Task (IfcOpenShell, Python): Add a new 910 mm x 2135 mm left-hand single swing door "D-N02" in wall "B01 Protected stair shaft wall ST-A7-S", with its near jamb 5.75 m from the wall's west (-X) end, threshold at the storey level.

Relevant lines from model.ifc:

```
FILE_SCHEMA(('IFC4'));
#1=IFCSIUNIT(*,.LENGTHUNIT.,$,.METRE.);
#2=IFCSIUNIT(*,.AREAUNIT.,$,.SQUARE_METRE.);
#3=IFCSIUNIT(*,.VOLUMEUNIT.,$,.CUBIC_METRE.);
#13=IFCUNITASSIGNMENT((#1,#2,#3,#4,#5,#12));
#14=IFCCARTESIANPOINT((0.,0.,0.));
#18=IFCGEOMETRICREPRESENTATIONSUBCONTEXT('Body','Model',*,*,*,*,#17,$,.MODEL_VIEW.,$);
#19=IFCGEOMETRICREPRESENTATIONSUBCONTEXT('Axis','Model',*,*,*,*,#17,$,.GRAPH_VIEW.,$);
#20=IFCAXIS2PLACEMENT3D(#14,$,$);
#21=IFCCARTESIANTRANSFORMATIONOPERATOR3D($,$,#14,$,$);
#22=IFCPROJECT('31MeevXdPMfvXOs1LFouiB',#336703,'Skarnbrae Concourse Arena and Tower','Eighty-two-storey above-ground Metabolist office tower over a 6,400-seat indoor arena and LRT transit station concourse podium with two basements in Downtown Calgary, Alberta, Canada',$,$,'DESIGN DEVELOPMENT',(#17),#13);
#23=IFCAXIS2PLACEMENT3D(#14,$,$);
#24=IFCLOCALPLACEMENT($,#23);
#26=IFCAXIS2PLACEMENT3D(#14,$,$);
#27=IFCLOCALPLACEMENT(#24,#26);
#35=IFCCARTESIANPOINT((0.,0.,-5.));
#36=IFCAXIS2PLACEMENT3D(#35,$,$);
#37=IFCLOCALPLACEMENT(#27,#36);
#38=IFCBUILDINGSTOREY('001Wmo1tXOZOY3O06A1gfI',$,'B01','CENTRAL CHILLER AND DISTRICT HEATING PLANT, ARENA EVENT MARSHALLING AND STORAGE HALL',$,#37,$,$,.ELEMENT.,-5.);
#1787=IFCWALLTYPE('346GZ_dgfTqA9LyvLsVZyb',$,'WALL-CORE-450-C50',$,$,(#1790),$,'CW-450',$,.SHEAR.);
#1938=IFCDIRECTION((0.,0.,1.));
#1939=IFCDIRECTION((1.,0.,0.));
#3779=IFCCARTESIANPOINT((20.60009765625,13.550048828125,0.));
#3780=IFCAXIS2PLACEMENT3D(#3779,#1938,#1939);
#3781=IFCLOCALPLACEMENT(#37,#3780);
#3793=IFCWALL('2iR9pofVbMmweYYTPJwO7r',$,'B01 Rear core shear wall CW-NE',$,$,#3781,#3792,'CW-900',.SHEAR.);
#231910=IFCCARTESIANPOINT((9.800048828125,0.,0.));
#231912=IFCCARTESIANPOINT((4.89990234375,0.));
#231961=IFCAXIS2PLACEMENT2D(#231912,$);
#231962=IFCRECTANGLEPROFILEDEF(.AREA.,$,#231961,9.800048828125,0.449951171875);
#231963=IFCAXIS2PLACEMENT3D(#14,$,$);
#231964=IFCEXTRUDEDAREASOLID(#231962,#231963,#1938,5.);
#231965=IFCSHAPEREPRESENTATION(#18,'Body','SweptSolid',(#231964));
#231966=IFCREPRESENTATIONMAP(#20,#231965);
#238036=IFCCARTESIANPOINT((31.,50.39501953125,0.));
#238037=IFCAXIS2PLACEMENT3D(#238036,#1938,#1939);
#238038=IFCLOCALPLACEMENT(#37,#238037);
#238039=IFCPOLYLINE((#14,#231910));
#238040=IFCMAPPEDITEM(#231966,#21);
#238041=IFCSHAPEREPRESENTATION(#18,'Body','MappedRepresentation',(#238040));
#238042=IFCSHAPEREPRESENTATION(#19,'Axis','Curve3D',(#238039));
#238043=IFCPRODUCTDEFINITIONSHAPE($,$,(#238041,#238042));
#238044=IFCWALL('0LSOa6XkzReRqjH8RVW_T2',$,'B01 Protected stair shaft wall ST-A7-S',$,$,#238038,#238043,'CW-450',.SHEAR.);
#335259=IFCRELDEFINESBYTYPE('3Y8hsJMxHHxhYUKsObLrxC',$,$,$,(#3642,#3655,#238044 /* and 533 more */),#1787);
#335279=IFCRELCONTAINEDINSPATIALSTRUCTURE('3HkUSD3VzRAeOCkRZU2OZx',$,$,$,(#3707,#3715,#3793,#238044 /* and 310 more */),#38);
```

```python
import numpy as np
import ifcopenshell
import ifcopenshell.api.feature
import ifcopenshell.api.geometry
import ifcopenshell.api.root
import ifcopenshell.api.spatial
import ifcopenshell.geom
import ifcopenshell.util.element
import ifcopenshell.util.placement
import ifcopenshell.util.representation
import ifcopenshell.util.shape
import ifcopenshell.util.unit

model = ifcopenshell.open("model.ifc")
unit_scale = ifcopenshell.util.unit.calculate_unit_scale(model)
settings = ifcopenshell.geom.settings()


def volume(element):
    """Net volume in cubic metres, openings subtracted."""
    shape = ifcopenshell.geom.create_shape(settings, element)
    return ifcopenshell.util.shape.get_volume(shape.geometry)


wall = model.by_guid("0LSOa6XkzReRqjH8RVW_T2")
storey = ifcopenshell.util.element.get_container(wall, ifc_class="IfcBuildingStorey")
context = ifcopenshell.util.representation.get_context(model, "Model", "Body", "MODEL_VIEW")
before = volume(wall)

width, height, from_end, sill = 0.91, 2.135, 5.75, 0.0  # metres

# The wall runs along its own X axis, and the end named is its -X end.
wall_shape = ifcopenshell.geom.create_shape(settings, wall)
x, y, z = ifcopenshell.util.shape.get_vertices(wall_shape.geometry).T
start = x.min() + from_end
face, thickness = float(y.min()), float(y.max() - y.min())
wall_matrix = ifcopenshell.util.placement.get_local_placement(wall.ObjectPlacement)
level = ifcopenshell.util.placement.get_local_placement(storey.ObjectPlacement)[2, 3]


def in_wall(x, y):
    """Placement at x, y metres in the wall's axes, at sill height."""
    matrix = wall_matrix.copy()
    matrix[:, 3] = wall_matrix @ np.array([x / unit_scale, y / unit_scale, 0.0, 1.0])
    matrix[2, 3] = level + sill / unit_scale
    return matrix


# Opening: a box that overshoots both wall faces by 50 mm.
opening = ifcopenshell.api.root.create_entity(model, ifc_class="IfcOpeningElement", predefined_type="OPENING")
box = ifcopenshell.api.geometry.add_wall_representation(
    model, context=context, length=width, height=height, thickness=thickness + 0.1
)
ifcopenshell.api.geometry.assign_representation(model, product=opening, representation=box)
ifcopenshell.api.geometry.edit_object_placement(model, product=opening, matrix=in_wall(start, face - 0.05), is_si=False)
ifcopenshell.api.feature.add_feature(model, feature=opening, element=wall)

door = ifcopenshell.api.root.create_entity(model, ifc_class="IfcDoor", name="D-N02", predefined_type="DOOR")
door.OverallWidth, door.OverallHeight = width / unit_scale, height / unit_scale
door.OperationType = "SINGLE_SWING_LEFT"
body = ifcopenshell.api.geometry.add_door_representation(
    model,
    context=context,
    overall_width=door.OverallWidth,
    overall_height=door.OverallHeight,
    operation_type="SINGLE_SWING_LEFT",
    lining_properties={"LiningDepth": thickness / unit_scale, "ThresholdDepth": thickness / unit_scale},
)
ifcopenshell.api.geometry.assign_representation(model, product=door, representation=body)
ifcopenshell.api.spatial.assign_container(model, products=[door], relating_structure=storey)
ifcopenshell.api.feature.add_filling(model, opening=opening, element=door)

# The lining spans the wall, so the door starts at the wall face.
ifcopenshell.api.geometry.edit_object_placement(model, product=door, matrix=in_wall(start, face), is_si=False)

after = volume(wall)

print(f"wall volume {before:.3f} -> {after:.3f} m3")

model.write("model_rev.ifc")
```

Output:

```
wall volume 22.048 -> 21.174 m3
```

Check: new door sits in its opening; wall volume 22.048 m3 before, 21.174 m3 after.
